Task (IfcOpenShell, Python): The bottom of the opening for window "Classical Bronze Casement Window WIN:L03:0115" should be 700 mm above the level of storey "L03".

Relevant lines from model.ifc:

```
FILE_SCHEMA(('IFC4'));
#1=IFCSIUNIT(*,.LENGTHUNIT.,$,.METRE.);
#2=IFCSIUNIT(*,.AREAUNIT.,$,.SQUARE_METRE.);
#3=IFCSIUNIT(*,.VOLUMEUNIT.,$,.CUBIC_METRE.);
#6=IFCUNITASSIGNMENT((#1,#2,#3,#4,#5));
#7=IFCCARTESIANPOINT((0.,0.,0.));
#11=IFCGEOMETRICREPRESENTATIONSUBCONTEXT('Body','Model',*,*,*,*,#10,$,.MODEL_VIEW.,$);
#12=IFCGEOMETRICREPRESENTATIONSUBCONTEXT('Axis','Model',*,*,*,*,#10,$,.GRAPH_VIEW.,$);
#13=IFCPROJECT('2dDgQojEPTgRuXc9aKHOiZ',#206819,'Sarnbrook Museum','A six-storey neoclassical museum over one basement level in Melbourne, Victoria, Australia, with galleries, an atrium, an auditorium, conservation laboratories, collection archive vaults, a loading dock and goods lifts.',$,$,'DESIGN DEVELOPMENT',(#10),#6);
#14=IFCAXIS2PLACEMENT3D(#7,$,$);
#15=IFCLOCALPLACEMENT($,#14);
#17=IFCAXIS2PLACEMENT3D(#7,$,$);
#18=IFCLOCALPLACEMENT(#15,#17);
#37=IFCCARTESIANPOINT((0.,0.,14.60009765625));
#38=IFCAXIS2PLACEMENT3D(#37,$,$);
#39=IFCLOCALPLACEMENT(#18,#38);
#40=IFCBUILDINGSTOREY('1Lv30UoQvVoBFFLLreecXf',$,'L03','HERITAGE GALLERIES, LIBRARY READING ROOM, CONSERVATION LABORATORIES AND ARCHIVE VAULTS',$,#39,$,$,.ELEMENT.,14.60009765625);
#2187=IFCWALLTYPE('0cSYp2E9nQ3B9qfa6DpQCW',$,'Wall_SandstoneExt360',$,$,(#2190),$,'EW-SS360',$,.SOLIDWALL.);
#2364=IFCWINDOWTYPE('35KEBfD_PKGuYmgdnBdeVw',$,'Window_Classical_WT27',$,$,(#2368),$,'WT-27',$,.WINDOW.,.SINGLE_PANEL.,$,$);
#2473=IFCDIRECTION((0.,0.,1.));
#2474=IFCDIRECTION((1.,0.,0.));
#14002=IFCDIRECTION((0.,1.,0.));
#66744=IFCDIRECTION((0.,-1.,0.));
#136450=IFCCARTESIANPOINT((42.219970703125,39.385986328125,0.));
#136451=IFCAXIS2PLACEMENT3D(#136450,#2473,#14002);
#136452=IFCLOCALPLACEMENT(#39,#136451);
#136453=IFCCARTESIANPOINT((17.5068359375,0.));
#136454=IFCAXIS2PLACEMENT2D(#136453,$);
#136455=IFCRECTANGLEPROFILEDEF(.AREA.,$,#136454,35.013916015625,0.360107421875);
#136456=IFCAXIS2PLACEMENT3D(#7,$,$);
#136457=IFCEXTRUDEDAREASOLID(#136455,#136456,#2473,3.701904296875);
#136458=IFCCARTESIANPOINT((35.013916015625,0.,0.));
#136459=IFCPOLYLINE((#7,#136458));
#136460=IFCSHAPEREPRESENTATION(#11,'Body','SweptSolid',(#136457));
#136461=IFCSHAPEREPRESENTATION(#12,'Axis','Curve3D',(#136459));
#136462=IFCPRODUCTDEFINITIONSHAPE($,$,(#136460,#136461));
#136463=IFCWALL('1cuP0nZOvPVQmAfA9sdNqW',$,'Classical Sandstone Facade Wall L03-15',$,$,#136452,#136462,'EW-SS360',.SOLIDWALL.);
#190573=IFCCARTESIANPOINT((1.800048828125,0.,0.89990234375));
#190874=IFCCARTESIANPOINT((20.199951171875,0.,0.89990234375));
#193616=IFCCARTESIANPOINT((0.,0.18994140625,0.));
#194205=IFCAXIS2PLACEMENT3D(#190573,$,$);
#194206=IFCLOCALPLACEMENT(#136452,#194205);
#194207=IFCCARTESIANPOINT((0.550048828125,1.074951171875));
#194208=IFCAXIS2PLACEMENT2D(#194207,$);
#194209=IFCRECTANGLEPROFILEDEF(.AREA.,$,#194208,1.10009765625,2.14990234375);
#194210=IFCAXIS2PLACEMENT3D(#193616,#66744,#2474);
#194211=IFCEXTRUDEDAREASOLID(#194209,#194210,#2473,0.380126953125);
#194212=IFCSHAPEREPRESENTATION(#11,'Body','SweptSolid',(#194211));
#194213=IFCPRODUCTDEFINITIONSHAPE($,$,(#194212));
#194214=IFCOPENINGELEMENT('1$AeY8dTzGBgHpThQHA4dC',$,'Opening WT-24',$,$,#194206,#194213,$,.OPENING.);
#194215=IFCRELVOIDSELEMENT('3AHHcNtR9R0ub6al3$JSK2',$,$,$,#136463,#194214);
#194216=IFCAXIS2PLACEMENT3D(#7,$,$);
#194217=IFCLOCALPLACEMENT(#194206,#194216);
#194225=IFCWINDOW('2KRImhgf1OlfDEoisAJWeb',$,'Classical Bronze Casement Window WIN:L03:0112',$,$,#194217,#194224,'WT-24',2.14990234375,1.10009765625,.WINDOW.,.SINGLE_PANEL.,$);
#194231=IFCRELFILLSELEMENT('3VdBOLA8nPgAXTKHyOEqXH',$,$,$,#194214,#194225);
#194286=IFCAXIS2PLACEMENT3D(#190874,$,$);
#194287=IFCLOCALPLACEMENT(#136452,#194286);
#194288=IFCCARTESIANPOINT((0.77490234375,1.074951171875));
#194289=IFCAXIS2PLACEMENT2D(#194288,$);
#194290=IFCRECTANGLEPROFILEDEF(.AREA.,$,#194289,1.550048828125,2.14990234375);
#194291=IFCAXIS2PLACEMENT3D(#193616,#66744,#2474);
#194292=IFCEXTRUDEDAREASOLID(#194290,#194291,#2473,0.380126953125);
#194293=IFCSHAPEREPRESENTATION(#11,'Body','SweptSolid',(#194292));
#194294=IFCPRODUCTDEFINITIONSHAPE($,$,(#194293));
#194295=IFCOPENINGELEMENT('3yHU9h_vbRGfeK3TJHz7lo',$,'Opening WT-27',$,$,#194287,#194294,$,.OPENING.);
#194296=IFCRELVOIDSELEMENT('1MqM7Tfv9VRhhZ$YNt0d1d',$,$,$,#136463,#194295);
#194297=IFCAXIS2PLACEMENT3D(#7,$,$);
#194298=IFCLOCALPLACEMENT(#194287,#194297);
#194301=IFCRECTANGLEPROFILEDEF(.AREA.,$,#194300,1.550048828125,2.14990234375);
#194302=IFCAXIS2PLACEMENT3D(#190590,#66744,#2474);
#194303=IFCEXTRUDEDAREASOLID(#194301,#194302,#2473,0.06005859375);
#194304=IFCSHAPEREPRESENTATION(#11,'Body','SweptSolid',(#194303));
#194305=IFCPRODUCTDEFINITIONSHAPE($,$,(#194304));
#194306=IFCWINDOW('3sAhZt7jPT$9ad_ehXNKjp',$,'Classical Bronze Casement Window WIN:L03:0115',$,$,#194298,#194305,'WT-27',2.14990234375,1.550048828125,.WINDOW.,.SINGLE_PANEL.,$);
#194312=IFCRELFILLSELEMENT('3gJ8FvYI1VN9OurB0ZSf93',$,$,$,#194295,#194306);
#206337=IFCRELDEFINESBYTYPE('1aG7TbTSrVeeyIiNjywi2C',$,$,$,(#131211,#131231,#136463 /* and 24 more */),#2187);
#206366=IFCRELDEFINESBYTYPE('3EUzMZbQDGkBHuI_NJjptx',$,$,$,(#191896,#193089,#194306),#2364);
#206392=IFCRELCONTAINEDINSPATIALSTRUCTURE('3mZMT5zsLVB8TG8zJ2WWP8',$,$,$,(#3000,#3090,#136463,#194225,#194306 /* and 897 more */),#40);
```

```python
import numpy as np
import ifcopenshell
import ifcopenshell.api.geometry
import ifcopenshell.geom
import ifcopenshell.util.element
import ifcopenshell.util.placement
import ifcopenshell.util.shape
import ifcopenshell.util.unit

model = ifcopenshell.open("model.ifc")
unit_scale = ifcopenshell.util.unit.calculate_unit_scale(model)

window = model.by_guid("3sAhZt7jPT$9ad_ehXNKjp")
opening = window.FillsVoids[0].RelatingOpeningElement
storey = ifcopenshell.util.element.get_container(window, ifc_class="IfcBuildingStorey")
level = ifcopenshell.util.placement.get_local_placement(storey.ObjectPlacement)[2, 3]

# The opening's origin need not be at the sill, so measure its lowest point.
shape = ifcopenshell.geom.create_shape(ifcopenshell.geom.settings(), opening)
bottom = ifcopenshell.util.shape.get_shape_bottom_elevation(shape, shape.geometry) / unit_scale
dz = level + 0.7 / unit_scale - bottom

shift = np.array([0.0, 0.0, dz])
# The window is placed relative to its opening, so it follows when the opening moves.
matrix = ifcopenshell.util.placement.get_local_placement(opening.ObjectPlacement)
matrix[:3, 3] += shift
ifcopenshell.api.geometry.edit_object_placement(
    model, product=opening, matrix=matrix, is_si=False, should_transform_children=True
)

print(f"moved by {dz * unit_scale:+.3f} m")

model.write("model-out.ifc")
```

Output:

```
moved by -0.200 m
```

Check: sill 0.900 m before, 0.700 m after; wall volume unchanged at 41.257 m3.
